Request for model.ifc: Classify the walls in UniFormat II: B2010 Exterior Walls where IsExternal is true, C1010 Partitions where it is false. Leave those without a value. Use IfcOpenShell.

First a look at what the model holds.

```python
import ifcopenshell
import ifcopenshell.util.element

model = ifcopenshell.open("model.ifc")
print(model.schema)
print("classifications:", [c.Name for c in model.by_type("IfcClassification")])
values = [ifcopenshell.util.element.get_pset(e, "Pset_WallCommon", "IsExternal") for e in model.by_type("IfcWall")]
for value in (True, False, None):
    print("IsExternal", value, values.count(value))
```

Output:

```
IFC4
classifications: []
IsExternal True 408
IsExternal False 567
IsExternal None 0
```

```python
import ifcopenshell
import ifcopenshell.api.classification
import ifcopenshell.util.element

model = ifcopenshell.open("model.ifc")

system = ifcopenshell.api.classification.add_classification(model, classification="UniFormat II")

walls = model.by_type("IfcWall")
external = {e: ifcopenshell.util.element.get_pset(e, "Pset_WallCommon", "IsExternal") for e in walls}
for flag, code, name in ((True, "B2010", "Exterior Walls"), (False, "C1010", "Partitions")):
    products = [e for e in walls if external[e] is flag]
    ifcopenshell.api.classification.add_reference(
        model, products=products, classification=system, identification=code, name=name
    )
    print(code, len(products))

model.write("model_edited.ifc")
```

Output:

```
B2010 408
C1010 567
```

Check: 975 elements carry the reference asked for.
